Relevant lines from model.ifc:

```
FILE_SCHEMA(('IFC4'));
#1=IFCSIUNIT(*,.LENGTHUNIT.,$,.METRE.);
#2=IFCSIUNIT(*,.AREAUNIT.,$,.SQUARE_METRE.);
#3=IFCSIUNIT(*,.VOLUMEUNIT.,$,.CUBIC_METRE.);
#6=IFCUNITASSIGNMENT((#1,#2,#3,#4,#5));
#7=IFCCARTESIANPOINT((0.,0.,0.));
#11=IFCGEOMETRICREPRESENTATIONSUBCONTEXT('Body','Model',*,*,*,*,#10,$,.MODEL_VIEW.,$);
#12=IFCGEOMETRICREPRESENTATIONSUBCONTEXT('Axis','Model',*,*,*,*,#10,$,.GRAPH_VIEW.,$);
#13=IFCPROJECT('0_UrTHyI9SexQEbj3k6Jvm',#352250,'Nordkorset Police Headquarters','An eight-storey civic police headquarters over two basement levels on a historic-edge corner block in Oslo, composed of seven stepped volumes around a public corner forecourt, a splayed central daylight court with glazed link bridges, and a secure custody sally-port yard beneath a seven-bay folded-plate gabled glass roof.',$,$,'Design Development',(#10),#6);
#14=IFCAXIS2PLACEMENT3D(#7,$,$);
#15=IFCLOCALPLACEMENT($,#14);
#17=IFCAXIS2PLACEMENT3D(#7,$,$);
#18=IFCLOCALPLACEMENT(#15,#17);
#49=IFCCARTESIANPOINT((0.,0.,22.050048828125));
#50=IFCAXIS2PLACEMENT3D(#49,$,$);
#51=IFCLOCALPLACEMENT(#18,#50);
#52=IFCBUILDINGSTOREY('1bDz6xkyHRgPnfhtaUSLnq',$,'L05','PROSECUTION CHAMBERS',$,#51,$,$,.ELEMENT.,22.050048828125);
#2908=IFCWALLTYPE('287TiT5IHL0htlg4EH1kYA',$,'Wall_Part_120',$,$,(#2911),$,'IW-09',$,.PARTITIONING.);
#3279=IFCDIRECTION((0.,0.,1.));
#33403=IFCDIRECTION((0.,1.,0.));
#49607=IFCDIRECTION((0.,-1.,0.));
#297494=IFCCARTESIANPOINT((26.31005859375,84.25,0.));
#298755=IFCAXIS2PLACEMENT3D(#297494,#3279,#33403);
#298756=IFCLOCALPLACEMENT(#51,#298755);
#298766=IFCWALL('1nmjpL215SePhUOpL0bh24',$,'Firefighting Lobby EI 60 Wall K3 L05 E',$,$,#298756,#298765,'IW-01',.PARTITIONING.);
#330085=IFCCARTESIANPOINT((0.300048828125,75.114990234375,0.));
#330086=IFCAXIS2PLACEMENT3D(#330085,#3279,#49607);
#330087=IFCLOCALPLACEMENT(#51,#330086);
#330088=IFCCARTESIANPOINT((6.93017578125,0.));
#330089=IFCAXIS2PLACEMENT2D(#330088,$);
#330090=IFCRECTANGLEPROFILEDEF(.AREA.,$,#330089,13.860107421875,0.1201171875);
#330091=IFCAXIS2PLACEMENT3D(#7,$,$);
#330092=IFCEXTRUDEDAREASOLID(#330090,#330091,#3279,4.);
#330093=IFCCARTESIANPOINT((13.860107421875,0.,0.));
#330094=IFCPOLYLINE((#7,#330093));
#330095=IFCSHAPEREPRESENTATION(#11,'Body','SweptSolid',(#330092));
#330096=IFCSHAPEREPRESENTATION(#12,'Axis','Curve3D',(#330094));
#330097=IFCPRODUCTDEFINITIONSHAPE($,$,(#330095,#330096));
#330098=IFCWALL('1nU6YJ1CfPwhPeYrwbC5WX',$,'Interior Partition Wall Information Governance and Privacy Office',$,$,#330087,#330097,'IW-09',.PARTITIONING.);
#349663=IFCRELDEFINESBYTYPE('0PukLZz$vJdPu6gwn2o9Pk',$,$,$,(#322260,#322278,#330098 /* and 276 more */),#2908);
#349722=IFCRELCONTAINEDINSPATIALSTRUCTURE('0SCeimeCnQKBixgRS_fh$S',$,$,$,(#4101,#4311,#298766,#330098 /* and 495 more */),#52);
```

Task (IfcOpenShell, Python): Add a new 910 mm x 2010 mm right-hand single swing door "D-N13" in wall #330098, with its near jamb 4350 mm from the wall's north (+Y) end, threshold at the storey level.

```python
import numpy as np
import ifcopenshell
import ifcopenshell.api.feature
import ifcopenshell.api.geometry
import ifcopenshell.api.root
import ifcopenshell.api.spatial
import ifcopenshell.geom
import ifcopenshell.util.element
import ifcopenshell.util.placement
import ifcopenshell.util.representation
import ifcopenshell.util.shape
import ifcopenshell.util.unit

model = ifcopenshell.open("model.ifc")
unit_scale = ifcopenshell.util.unit.calculate_unit_scale(model)
settings = ifcopenshell.geom.settings()


def volume(element):
    """Net volume in cubic metres, openings subtracted."""
    shape = ifcopenshell.geom.create_shape(settings, element)
    return ifcopenshell.util.shape.get_volume(shape.geometry)


wall = model.by_guid("1nU6YJ1CfPwhPeYrwbC5WX")
storey = ifcopenshell.util.element.get_container(wall, ifc_class="IfcBuildingStorey")
context = ifcopenshell.util.representation.get_context(model, "Model", "Body", "MODEL_VIEW")
before = volume(wall)

width, height, from_end, sill = 0.91, 2.01, 4.35, 0.0  # metres

# The wall runs along its own X axis, and the end named is its -X end.
wall_shape = ifcopenshell.geom.create_shape(settings, wall)
x, y, z = ifcopenshell.util.shape.get_vertices(wall_shape.geometry).T
start = x.min() + from_end
face, thickness = float(y.min()), float(y.max() - y.min())
wall_matrix = ifcopenshell.util.placement.get_local_placement(wall.ObjectPlacement)
level = ifcopenshell.util.placement.get_local_placement(storey.ObjectPlacement)[2, 3]


def in_wall(x, y):
    """Placement at x, y metres in the wall's axes, at sill height."""
    matrix = wall_matrix.copy()
    matrix[:, 3] = wall_matrix @ np.array([x / unit_scale, y / unit_scale, 0.0, 1.0])
    matrix[2, 3] = level + sill / unit_scale
    return matrix


# Opening: a box that overshoots both wall faces by 50 mm.
opening = ifcopenshell.api.root.create_entity(model, ifc_class="IfcOpeningElement", predefined_type="OPENING")
box = ifcopenshell.api.geometry.add_wall_representation(
    model, context=context, length=width, height=height, thickness=thickness + 0.1
)
ifcopenshell.api.geometry.assign_representation(model, product=opening, representation=box)
ifcopenshell.api.geometry.edit_object_placement(model, product=opening, matrix=in_wall(start, face - 0.05), is_si=False)
ifcopenshell.api.feature.add_feature(model, feature=opening, element=wall)

door = ifcopenshell.api.root.create_entity(model, ifc_class="IfcDoor", name="D-N13", predefined_type="DOOR")
door.OverallWidth, door.OverallHeight = width / unit_scale, height / unit_scale
door.OperationType = "SINGLE_SWING_RIGHT"
body = ifcopenshell.api.geometry.add_door_representation(
    model,
    context=context,
    overall_width=door.OverallWidth,
    overall_height=door.OverallHeight,
    operation_type="SINGLE_SWING_RIGHT",
    lining_properties={"LiningDepth": thickness / unit_scale, "ThresholdDepth": thickness / unit_scale},
)
ifcopenshell.api.geometry.assign_representation(model, product=door, representation=body)
ifcopenshell.api.spatial.assign_container(model, products=[door], relating_structure=storey)
ifcopenshell.api.feature.add_filling(model, opening=opening, element=door)

# The lining spans the wall, so the door starts at the wall face.
ifcopenshell.api.geometry.edit_object_placement(model, product=door, matrix=in_wall(start, face), is_si=False)

after = volume(wall)

print(f"wall volume {before:.3f} -> {after:.3f} m3")

model.write("model_rev.ifc")
```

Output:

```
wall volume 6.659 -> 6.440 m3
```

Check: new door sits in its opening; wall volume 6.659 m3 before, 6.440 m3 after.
